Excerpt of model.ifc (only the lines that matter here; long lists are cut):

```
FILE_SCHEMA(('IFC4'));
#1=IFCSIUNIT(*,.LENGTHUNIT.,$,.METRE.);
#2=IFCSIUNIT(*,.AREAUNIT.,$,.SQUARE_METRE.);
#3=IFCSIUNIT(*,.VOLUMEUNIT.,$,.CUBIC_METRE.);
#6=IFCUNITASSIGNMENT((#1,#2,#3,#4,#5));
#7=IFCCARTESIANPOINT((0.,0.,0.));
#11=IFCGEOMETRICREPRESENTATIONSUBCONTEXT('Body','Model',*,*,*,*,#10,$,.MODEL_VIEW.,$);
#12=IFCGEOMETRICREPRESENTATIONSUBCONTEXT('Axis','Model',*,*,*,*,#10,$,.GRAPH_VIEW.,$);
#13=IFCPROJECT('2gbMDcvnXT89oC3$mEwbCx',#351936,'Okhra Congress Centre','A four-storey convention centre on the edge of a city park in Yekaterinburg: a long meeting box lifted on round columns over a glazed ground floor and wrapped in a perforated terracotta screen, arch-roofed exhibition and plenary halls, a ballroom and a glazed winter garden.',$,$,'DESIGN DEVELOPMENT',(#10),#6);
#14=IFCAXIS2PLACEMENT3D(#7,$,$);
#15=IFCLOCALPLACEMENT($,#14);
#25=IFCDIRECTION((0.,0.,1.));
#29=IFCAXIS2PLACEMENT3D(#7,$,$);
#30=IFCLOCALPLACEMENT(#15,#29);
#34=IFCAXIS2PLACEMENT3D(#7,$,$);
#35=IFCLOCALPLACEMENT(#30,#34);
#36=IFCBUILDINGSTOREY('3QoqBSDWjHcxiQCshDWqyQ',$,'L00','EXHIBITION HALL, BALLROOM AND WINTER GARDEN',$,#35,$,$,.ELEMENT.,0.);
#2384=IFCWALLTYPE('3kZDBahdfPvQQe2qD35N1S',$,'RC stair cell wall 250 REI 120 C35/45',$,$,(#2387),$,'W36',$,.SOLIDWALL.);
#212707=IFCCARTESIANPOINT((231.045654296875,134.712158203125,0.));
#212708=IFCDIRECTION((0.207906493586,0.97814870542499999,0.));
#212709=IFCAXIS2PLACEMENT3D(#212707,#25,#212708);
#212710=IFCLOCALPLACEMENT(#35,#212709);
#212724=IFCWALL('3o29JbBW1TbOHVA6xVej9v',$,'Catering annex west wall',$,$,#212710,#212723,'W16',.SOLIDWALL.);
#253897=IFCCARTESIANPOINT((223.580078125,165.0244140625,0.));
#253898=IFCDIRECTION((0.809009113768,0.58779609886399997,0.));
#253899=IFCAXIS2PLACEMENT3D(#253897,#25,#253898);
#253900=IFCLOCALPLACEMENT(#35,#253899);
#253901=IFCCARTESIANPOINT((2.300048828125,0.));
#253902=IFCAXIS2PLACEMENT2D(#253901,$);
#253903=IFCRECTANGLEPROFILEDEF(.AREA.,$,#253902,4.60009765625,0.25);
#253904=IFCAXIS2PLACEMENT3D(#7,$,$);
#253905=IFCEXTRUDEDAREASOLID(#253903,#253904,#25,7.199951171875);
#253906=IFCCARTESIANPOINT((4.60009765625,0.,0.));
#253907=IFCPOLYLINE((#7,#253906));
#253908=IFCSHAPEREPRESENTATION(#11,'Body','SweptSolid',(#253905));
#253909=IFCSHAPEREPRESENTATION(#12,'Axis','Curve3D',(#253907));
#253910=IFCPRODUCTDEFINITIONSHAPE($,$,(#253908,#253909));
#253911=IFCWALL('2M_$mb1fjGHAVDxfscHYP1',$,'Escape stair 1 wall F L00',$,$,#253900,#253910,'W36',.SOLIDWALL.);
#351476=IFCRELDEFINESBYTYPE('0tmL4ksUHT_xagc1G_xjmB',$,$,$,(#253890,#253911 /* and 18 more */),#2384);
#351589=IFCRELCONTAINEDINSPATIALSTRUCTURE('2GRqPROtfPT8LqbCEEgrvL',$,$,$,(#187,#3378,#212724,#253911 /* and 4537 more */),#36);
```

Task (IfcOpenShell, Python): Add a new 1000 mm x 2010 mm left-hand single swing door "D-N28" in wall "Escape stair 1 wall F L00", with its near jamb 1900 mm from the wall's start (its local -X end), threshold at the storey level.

```python
import numpy as np
import ifcopenshell
import ifcopenshell.api.feature
import ifcopenshell.api.geometry
import ifcopenshell.api.root
import ifcopenshell.api.spatial
import ifcopenshell.geom
import ifcopenshell.util.element
import ifcopenshell.util.placement
import ifcopenshell.util.representation
import ifcopenshell.util.shape
import ifcopenshell.util.unit

model = ifcopenshell.open("model.ifc")
unit_scale = ifcopenshell.util.unit.calculate_unit_scale(model)
settings = ifcopenshell.geom.settings()


def volume(element):
    """Net volume in cubic metres, openings subtracted."""
    shape = ifcopenshell.geom.create_shape(settings, element)
    return ifcopenshell.util.shape.get_volume(shape.geometry)


wall = model.by_guid("2M_$mb1fjGHAVDxfscHYP1")
storey = ifcopenshell.util.element.get_container(wall, ifc_class="IfcBuildingStorey")
context = ifcopenshell.util.representation.get_context(model, "Model", "Body", "MODEL_VIEW")
before = volume(wall)

width, height, from_end, sill = 1, 2.01, 1.9, 0.0  # metres

# The wall runs along its own X axis, and the end named is its -X end.
wall_shape = ifcopenshell.geom.create_shape(settings, wall)
x, y, z = ifcopenshell.util.shape.get_vertices(wall_shape.geometry).T
start = x.min() + from_end
face, thickness = float(y.min()), float(y.max() - y.min())
wall_matrix = ifcopenshell.util.placement.get_local_placement(wall.ObjectPlacement)
level = ifcopenshell.util.placement.get_local_placement(storey.ObjectPlacement)[2, 3]


def in_wall(x, y):
    """Placement at x, y metres in the wall's axes, at sill height."""
    matrix = wall_matrix.copy()
    matrix[:, 3] = wall_matrix @ np.array([x / unit_scale, y / unit_scale, 0.0, 1.0])
    matrix[2, 3] = level + sill / unit_scale
    return matrix


# Opening: a box that overshoots both wall faces by 50 mm.
opening = ifcopenshell.api.root.create_entity(model, ifc_class="IfcOpeningElement", predefined_type="OPENING")
box = ifcopenshell.api.geometry.add_wall_representation(
    model, context=context, length=width, height=height, thickness=thickness + 0.1
)
ifcopenshell.api.geometry.assign_representation(model, product=opening, representation=box)
ifcopenshell.api.geometry.edit_object_placement(model, product=opening, matrix=in_wall(start, face - 0.05), is_si=False)
ifcopenshell.api.feature.add_feature(model, feature=opening, element=wall)

door = ifcopenshell.api.root.create_entity(model, ifc_class="IfcDoor", name="D-N28", predefined_type="DOOR")
door.OverallWidth, door.OverallHeight = width / unit_scale, height / unit_scale
door.OperationType = "SINGLE_SWING_LEFT"
body = ifcopenshell.api.geometry.add_door_representation(
    model,
    context=context,
    overall_width=door.OverallWidth,
    overall_height=door.OverallHeight,
    operation_type="SINGLE_SWING_LEFT",
    lining_properties={"LiningDepth": thickness / unit_scale, "ThresholdDepth": thickness / unit_scale},
)
ifcopenshell.api.geometry.assign_representation(model, product=door, representation=body)
ifcopenshell.api.spatial.assign_container(model, products=[door], relating_structure=storey)
ifcopenshell.api.feature.add_filling(model, opening=opening, element=door)

# The lining spans the wall, so the door starts at the wall face.
ifcopenshell.api.geometry.edit_object_placement(model, product=door, matrix=in_wall(start, face), is_si=False)

after = volume(wall)

print(f"wall volume {before:.3f} -> {after:.3f} m3")

model.write("model_rev.ifc")
```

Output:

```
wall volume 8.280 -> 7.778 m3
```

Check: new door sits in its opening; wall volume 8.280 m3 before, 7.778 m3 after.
